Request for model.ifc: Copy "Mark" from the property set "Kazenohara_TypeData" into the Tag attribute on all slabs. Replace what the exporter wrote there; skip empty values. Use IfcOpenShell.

First a look at what the model holds.

```python
import ifcopenshell
import ifcopenshell.util.element

model = ifcopenshell.open("model.ifc")
print(model.schema)
slabs = model.by_type("IfcSlab")
print(len(slabs), "slabs")
for e in slabs[:8]:
    source = ifcopenshell.util.element.get_pset(e, "Kazenohara_TypeData", "Mark")
    target = e.Tag
    print(e.id(), repr(source), repr(target), sep=" | ")
```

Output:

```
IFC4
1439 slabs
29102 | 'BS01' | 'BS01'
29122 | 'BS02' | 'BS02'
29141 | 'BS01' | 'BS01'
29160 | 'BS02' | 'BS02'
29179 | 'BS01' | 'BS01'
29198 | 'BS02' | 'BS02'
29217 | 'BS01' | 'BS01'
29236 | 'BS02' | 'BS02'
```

```python
import ifcopenshell
import ifcopenshell.util.element

model = ifcopenshell.open("model.ifc")

count = 0
for e in model.by_type("IfcSlab"):
    value = ifcopenshell.util.element.get_pset(e, "Kazenohara_TypeData", "Mark")
    current = e.Tag
    if not value or not value.strip() or current == value:
        continue
    e.Tag = value
    count += 1

print(count, "slabs updated")

model.write("model-out.ifc")
```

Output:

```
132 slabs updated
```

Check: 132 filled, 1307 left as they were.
